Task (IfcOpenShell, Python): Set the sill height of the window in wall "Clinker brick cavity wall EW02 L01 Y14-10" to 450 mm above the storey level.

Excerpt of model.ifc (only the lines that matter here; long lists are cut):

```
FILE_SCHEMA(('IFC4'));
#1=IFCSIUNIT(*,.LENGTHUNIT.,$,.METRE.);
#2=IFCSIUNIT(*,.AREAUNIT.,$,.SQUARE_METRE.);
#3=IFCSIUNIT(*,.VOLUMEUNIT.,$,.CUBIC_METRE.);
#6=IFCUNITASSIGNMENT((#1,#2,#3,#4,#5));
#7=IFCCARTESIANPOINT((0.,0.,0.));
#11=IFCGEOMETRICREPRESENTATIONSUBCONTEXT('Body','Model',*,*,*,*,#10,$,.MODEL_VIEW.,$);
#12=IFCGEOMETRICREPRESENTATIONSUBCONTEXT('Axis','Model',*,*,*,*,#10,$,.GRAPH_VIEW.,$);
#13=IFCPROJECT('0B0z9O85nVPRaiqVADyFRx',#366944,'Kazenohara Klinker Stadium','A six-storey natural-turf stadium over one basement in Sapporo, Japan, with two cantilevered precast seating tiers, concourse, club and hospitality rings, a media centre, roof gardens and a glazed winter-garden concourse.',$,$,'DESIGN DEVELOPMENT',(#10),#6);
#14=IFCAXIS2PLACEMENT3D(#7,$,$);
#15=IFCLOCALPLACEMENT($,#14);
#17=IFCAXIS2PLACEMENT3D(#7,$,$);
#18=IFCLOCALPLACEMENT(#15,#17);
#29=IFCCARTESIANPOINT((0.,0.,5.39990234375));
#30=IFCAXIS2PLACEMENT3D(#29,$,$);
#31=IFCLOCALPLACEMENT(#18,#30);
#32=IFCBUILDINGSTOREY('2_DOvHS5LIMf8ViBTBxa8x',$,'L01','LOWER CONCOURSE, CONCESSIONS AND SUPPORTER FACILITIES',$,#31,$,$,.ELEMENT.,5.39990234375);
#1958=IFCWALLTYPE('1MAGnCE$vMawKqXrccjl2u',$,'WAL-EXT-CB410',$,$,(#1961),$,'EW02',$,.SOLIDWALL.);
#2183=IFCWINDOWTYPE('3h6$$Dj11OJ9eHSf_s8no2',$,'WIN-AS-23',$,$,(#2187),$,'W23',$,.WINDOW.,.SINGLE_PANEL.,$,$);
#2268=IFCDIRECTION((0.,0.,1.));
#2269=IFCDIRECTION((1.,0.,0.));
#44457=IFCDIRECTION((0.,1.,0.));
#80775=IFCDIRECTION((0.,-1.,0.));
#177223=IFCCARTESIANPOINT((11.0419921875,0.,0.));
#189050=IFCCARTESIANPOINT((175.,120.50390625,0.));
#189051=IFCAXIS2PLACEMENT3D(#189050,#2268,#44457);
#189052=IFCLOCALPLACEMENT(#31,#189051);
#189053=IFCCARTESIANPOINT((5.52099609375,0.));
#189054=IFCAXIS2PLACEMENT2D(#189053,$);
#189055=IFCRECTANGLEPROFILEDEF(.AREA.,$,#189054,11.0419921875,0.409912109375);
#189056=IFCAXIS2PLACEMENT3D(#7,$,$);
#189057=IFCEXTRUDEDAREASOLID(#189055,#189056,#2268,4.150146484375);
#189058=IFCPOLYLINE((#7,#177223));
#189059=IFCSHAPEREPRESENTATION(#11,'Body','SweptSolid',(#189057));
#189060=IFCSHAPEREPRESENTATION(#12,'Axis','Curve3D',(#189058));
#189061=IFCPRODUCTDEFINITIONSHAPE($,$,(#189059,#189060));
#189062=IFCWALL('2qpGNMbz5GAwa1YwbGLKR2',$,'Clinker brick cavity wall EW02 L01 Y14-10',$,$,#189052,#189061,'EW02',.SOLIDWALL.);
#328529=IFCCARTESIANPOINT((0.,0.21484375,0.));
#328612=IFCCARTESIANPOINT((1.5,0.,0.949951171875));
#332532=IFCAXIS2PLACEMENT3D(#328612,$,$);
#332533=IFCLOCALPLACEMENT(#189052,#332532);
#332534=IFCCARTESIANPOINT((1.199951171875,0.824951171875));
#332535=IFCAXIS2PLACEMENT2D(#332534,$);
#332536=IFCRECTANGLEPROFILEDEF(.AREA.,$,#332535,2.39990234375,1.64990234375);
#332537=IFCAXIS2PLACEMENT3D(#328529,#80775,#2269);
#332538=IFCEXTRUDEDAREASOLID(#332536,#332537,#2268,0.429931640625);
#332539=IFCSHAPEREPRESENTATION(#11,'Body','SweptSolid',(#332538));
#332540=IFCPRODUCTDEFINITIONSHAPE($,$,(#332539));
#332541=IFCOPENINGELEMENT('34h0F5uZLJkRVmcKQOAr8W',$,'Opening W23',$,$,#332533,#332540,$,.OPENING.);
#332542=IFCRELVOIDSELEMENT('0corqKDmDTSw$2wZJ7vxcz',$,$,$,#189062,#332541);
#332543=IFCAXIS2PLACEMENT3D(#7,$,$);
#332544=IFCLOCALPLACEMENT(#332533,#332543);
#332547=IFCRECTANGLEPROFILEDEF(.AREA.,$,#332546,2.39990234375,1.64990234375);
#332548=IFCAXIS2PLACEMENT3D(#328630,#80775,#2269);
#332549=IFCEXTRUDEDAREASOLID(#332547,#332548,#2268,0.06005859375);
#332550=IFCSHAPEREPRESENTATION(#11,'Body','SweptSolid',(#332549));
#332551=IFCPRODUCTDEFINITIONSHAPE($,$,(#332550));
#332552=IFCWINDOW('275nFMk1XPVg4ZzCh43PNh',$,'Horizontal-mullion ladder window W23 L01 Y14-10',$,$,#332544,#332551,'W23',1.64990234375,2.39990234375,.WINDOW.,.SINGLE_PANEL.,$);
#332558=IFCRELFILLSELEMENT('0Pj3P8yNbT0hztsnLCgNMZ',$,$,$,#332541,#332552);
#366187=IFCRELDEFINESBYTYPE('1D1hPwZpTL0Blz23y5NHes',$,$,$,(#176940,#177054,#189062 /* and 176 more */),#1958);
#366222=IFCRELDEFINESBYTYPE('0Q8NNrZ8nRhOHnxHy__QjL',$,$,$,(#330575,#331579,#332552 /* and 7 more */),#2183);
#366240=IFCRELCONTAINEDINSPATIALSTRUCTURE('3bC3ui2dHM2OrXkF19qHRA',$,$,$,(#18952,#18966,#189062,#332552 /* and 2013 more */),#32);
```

```python
import numpy as np
import ifcopenshell
import ifcopenshell.api.geometry
import ifcopenshell.geom
import ifcopenshell.util.element
import ifcopenshell.util.placement
import ifcopenshell.util.shape
import ifcopenshell.util.unit

model = ifcopenshell.open("model.ifc")
unit_scale = ifcopenshell.util.unit.calculate_unit_scale(model)

window = model.by_guid("275nFMk1XPVg4ZzCh43PNh")
opening = window.FillsVoids[0].RelatingOpeningElement
storey = ifcopenshell.util.element.get_container(window, ifc_class="IfcBuildingStorey")
level = ifcopenshell.util.placement.get_local_placement(storey.ObjectPlacement)[2, 3]

# The opening's origin need not be at the sill, so measure its lowest point.
shape = ifcopenshell.geom.create_shape(ifcopenshell.geom.settings(), opening)
bottom = ifcopenshell.util.shape.get_shape_bottom_elevation(shape, shape.geometry) / unit_scale
dz = level + 0.45 - bottom

shift = np.array([0.0, 0.0, dz])
# The window is placed relative to its opening, so it follows when the opening moves.
matrix = ifcopenshell.util.placement.get_local_placement(opening.ObjectPlacement)
matrix[:3, 3] += shift
ifcopenshell.api.geometry.edit_object_placement(
    model, product=opening, matrix=matrix, is_si=False, should_transform_children=True
)

print(f"moved by {dz * unit_scale:+.3f} m")

model.write("model-out.ifc")
```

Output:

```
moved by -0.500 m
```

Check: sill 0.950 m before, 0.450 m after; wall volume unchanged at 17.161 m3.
